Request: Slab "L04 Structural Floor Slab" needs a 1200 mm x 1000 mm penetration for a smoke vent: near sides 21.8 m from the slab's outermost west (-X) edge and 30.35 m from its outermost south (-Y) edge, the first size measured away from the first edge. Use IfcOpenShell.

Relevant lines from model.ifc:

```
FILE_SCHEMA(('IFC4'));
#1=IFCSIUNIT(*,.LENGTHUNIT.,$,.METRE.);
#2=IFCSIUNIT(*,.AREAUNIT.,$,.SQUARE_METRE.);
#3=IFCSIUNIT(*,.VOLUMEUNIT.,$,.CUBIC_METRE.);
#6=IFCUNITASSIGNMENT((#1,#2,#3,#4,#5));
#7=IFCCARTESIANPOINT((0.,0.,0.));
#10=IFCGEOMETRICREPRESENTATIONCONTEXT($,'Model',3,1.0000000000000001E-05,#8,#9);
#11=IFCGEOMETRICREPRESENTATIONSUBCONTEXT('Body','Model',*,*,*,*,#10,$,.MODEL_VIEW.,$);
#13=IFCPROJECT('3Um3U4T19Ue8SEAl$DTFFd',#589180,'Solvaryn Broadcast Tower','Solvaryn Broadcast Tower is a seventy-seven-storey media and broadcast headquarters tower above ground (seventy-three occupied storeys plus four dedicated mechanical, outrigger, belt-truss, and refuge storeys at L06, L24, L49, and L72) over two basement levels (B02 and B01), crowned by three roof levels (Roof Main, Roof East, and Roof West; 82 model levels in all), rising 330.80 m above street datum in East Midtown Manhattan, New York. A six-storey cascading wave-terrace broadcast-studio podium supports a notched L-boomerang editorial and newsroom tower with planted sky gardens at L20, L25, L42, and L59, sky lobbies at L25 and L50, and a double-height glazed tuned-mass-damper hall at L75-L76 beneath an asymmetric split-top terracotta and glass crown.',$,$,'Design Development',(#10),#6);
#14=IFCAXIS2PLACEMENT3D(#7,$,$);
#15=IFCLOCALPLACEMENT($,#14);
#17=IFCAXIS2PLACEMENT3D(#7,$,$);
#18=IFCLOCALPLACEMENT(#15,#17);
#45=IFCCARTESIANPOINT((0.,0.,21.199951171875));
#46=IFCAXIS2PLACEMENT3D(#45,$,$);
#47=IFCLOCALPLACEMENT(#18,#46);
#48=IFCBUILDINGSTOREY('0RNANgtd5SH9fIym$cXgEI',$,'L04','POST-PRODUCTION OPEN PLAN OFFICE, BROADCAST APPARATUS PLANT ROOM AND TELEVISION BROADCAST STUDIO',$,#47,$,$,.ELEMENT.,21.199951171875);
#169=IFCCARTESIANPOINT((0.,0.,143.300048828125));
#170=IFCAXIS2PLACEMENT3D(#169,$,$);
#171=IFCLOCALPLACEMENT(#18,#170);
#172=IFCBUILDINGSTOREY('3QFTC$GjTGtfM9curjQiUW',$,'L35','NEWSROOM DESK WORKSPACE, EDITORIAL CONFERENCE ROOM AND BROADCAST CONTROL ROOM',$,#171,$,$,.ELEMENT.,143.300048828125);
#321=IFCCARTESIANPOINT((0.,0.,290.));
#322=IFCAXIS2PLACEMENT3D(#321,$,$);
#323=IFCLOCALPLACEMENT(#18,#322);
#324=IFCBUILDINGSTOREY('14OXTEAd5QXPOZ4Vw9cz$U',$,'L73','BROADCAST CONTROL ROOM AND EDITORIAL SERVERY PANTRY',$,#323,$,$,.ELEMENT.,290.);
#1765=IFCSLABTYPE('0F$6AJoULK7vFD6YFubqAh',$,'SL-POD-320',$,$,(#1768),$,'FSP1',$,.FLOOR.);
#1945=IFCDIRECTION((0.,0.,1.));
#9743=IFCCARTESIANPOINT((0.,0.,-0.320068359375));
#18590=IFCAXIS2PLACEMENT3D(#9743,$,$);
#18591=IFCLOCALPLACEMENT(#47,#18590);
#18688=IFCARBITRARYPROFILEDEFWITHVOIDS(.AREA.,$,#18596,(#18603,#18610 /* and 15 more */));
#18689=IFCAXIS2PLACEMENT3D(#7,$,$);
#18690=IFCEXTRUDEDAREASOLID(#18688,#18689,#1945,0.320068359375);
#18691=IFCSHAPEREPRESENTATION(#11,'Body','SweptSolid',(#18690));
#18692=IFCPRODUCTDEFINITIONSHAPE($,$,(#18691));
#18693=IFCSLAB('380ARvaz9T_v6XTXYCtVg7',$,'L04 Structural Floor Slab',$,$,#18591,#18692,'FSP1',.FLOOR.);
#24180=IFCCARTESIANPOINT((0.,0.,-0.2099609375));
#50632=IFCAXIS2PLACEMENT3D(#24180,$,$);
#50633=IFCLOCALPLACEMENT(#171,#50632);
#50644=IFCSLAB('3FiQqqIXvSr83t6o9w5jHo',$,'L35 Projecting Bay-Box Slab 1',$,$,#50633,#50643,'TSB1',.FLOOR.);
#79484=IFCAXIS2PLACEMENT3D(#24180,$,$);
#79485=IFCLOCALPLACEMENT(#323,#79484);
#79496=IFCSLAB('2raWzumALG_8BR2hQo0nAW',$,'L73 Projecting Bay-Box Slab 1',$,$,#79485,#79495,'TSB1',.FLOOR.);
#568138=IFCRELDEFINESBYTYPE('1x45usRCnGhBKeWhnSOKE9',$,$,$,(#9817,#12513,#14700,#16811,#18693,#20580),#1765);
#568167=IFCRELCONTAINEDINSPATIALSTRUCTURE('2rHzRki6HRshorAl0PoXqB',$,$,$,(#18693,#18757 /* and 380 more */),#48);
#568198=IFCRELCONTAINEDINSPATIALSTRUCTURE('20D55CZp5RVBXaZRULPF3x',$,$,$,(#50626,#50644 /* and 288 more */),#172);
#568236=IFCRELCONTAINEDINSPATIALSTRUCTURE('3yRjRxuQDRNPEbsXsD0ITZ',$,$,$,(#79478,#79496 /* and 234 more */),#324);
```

```python
import numpy as np
import ifcopenshell
import ifcopenshell.api.feature
import ifcopenshell.api.geometry
import ifcopenshell.api.root
import ifcopenshell.geom
import ifcopenshell.util.placement
import ifcopenshell.util.representation
import ifcopenshell.util.shape
import ifcopenshell.util.unit

model = ifcopenshell.open("model.ifc")
unit_scale = ifcopenshell.util.unit.calculate_unit_scale(model)
settings = ifcopenshell.geom.settings()


def volume(element):
    """Net volume in cubic metres, openings subtracted."""
    shape = ifcopenshell.geom.create_shape(settings, element)
    return ifcopenshell.util.shape.get_volume(shape.geometry)


slab = model.by_guid("380ARvaz9T_v6XTXYCtVg7")
before = volume(slab)

# Extent in the slab's own axes, in metres. The edges named are its -X and -Y sides.
slab_shape = ifcopenshell.geom.create_shape(settings, slab)
vertices = ifcopenshell.util.shape.get_vertices(slab_shape.geometry)
x_min, y_min, bottom = vertices.min(axis=0)
top = vertices[:, 2].max()

opening = ifcopenshell.api.root.create_entity(model, ifc_class="IfcOpeningElement", name="Smoke vent opening", predefined_type="OPENING")
context = ifcopenshell.util.representation.get_context(model, "Model", "Body", "MODEL_VIEW")
width, depth = 1.2, 1
outline = [(0.0, 0.0), (width, 0.0), (width, depth), (0.0, depth), (0.0, 0.0)]
# Overshoot both faces by 50 mm so the cut is clean.
shape = ifcopenshell.api.geometry.add_slab_representation(
    model, context=context, depth=top - bottom + 0.1, polyline=outline
)
ifcopenshell.api.geometry.assign_representation(model, product=opening, representation=shape)

matrix = ifcopenshell.util.placement.get_local_placement(slab.ObjectPlacement)
matrix[:, 3] = matrix @ np.append(np.array([x_min + 21.8, y_min + 30.35, bottom - 0.05]) / unit_scale, 1.0)
ifcopenshell.api.geometry.edit_object_placement(model, product=opening, matrix=matrix, is_si=False)
ifcopenshell.api.feature.add_feature(model, feature=opening, element=slab)

after = volume(slab)

print(f"slab volume {before:.3f} -> {after:.3f} m3")

model.write("model_rev.ifc")
```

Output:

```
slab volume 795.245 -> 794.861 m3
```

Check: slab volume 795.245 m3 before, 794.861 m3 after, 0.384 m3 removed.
